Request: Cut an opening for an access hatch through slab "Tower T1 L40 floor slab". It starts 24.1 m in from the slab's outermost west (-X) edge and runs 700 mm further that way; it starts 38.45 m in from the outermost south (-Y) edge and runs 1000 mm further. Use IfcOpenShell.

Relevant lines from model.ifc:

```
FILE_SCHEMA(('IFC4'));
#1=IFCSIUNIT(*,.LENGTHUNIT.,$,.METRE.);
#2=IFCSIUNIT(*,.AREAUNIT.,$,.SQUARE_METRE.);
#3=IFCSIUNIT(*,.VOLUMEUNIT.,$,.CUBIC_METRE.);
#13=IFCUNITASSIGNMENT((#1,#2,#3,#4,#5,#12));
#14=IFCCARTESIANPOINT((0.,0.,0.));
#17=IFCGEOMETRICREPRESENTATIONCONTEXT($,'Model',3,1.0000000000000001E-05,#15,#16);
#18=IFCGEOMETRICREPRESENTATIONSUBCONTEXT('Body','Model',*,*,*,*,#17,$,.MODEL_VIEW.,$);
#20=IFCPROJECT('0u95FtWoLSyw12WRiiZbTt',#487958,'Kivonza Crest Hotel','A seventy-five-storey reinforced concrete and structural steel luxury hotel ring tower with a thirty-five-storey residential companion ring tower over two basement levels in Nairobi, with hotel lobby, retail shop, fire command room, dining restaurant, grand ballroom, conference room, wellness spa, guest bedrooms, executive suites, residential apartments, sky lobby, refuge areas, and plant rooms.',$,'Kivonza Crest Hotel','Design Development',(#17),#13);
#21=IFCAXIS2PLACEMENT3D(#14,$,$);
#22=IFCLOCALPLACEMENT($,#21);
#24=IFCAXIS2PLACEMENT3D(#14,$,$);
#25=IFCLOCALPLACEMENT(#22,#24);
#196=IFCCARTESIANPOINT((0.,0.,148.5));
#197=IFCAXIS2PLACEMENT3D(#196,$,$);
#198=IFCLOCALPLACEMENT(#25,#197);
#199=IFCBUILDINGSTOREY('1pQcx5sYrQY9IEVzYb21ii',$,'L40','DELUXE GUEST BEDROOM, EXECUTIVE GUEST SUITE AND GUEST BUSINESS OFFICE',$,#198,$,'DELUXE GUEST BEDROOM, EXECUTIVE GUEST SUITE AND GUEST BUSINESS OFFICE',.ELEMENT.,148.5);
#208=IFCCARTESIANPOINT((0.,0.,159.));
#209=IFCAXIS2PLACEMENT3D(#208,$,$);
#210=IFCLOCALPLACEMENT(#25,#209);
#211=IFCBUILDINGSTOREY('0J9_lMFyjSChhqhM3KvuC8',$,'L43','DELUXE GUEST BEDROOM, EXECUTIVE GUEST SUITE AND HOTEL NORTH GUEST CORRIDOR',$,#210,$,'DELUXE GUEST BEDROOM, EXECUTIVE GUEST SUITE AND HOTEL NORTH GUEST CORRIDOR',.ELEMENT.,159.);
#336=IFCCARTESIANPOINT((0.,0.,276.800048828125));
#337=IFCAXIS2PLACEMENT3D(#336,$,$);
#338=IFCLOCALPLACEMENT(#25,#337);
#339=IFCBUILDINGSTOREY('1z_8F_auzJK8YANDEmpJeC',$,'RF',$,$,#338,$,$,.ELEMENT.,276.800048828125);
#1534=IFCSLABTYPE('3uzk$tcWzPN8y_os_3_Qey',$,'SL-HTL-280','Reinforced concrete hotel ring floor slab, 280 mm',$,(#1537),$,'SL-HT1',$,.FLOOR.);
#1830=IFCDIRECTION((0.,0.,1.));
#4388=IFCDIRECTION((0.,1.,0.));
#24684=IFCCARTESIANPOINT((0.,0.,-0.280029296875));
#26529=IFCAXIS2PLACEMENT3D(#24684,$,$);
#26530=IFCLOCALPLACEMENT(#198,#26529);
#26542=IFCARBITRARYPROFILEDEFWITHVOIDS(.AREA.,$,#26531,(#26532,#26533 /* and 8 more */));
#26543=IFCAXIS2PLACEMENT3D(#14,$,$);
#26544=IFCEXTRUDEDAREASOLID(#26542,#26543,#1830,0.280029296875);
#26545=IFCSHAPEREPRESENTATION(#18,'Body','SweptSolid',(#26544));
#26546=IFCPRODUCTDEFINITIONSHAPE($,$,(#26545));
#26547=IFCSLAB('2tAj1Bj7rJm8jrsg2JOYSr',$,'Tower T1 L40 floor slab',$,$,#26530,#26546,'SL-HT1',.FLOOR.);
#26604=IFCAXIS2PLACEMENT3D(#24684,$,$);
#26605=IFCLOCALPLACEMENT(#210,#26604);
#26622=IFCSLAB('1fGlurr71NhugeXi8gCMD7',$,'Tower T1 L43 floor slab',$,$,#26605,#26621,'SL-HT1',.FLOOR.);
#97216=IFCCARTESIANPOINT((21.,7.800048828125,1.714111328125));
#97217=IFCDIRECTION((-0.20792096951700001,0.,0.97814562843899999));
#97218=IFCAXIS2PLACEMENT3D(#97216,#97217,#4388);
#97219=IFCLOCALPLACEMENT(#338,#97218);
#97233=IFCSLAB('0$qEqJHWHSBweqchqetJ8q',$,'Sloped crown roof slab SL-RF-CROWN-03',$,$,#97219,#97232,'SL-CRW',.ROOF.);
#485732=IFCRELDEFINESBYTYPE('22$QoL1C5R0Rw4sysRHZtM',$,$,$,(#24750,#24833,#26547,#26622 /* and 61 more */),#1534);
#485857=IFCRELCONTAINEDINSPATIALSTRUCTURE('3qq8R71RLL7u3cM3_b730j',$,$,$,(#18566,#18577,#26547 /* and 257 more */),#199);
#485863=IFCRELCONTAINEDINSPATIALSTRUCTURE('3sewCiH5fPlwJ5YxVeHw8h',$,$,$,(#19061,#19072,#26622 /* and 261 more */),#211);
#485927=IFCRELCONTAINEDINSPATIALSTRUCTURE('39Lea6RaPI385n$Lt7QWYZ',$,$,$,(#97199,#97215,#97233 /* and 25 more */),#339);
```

```python
import numpy as np
import ifcopenshell
import ifcopenshell.api.feature
import ifcopenshell.api.geometry
import ifcopenshell.api.root
import ifcopenshell.geom
import ifcopenshell.util.placement
import ifcopenshell.util.representation
import ifcopenshell.util.shape
import ifcopenshell.util.unit

model = ifcopenshell.open("model.ifc")
unit_scale = ifcopenshell.util.unit.calculate_unit_scale(model)
settings = ifcopenshell.geom.settings()


def volume(element):
    """Net volume in cubic metres, openings subtracted."""
    shape = ifcopenshell.geom.create_shape(settings, element)
    return ifcopenshell.util.shape.get_volume(shape.geometry)


slab = model.by_id(26547)
before = volume(slab)

# Extent in the slab's own axes, in metres. The edges named are its -X and -Y sides.
slab_shape = ifcopenshell.geom.create_shape(settings, slab)
vertices = ifcopenshell.util.shape.get_vertices(slab_shape.geometry)
x_min, y_min, bottom = vertices.min(axis=0)
top = vertices[:, 2].max()

opening = ifcopenshell.api.root.create_entity(model, ifc_class="IfcOpeningElement", name="Access hatch opening", predefined_type="OPENING")
context = ifcopenshell.util.representation.get_context(model, "Model", "Body", "MODEL_VIEW")
width, depth = 0.7, 1
outline = [(0.0, 0.0), (width, 0.0), (width, depth), (0.0, depth), (0.0, 0.0)]
# Overshoot both faces by 50 mm so the cut is clean.
shape = ifcopenshell.api.geometry.add_slab_representation(
    model, context=context, depth=top - bottom + 0.1, polyline=outline
)
ifcopenshell.api.geometry.assign_representation(model, product=opening, representation=shape)

matrix = ifcopenshell.util.placement.get_local_placement(slab.ObjectPlacement)
matrix[:, 3] = matrix @ np.append(np.array([x_min + 24.1, y_min + 38.45, bottom - 0.05]) / unit_scale, 1.0)
ifcopenshell.api.geometry.edit_object_placement(model, product=opening, matrix=matrix, is_si=False)
ifcopenshell.api.feature.add_feature(model, feature=opening, element=slab)

after = volume(slab)

print(f"slab volume {before:.3f} -> {after:.3f} m3")

model.write("model_edited.ifc")
```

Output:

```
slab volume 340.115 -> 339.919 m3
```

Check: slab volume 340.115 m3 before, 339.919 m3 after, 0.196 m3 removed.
